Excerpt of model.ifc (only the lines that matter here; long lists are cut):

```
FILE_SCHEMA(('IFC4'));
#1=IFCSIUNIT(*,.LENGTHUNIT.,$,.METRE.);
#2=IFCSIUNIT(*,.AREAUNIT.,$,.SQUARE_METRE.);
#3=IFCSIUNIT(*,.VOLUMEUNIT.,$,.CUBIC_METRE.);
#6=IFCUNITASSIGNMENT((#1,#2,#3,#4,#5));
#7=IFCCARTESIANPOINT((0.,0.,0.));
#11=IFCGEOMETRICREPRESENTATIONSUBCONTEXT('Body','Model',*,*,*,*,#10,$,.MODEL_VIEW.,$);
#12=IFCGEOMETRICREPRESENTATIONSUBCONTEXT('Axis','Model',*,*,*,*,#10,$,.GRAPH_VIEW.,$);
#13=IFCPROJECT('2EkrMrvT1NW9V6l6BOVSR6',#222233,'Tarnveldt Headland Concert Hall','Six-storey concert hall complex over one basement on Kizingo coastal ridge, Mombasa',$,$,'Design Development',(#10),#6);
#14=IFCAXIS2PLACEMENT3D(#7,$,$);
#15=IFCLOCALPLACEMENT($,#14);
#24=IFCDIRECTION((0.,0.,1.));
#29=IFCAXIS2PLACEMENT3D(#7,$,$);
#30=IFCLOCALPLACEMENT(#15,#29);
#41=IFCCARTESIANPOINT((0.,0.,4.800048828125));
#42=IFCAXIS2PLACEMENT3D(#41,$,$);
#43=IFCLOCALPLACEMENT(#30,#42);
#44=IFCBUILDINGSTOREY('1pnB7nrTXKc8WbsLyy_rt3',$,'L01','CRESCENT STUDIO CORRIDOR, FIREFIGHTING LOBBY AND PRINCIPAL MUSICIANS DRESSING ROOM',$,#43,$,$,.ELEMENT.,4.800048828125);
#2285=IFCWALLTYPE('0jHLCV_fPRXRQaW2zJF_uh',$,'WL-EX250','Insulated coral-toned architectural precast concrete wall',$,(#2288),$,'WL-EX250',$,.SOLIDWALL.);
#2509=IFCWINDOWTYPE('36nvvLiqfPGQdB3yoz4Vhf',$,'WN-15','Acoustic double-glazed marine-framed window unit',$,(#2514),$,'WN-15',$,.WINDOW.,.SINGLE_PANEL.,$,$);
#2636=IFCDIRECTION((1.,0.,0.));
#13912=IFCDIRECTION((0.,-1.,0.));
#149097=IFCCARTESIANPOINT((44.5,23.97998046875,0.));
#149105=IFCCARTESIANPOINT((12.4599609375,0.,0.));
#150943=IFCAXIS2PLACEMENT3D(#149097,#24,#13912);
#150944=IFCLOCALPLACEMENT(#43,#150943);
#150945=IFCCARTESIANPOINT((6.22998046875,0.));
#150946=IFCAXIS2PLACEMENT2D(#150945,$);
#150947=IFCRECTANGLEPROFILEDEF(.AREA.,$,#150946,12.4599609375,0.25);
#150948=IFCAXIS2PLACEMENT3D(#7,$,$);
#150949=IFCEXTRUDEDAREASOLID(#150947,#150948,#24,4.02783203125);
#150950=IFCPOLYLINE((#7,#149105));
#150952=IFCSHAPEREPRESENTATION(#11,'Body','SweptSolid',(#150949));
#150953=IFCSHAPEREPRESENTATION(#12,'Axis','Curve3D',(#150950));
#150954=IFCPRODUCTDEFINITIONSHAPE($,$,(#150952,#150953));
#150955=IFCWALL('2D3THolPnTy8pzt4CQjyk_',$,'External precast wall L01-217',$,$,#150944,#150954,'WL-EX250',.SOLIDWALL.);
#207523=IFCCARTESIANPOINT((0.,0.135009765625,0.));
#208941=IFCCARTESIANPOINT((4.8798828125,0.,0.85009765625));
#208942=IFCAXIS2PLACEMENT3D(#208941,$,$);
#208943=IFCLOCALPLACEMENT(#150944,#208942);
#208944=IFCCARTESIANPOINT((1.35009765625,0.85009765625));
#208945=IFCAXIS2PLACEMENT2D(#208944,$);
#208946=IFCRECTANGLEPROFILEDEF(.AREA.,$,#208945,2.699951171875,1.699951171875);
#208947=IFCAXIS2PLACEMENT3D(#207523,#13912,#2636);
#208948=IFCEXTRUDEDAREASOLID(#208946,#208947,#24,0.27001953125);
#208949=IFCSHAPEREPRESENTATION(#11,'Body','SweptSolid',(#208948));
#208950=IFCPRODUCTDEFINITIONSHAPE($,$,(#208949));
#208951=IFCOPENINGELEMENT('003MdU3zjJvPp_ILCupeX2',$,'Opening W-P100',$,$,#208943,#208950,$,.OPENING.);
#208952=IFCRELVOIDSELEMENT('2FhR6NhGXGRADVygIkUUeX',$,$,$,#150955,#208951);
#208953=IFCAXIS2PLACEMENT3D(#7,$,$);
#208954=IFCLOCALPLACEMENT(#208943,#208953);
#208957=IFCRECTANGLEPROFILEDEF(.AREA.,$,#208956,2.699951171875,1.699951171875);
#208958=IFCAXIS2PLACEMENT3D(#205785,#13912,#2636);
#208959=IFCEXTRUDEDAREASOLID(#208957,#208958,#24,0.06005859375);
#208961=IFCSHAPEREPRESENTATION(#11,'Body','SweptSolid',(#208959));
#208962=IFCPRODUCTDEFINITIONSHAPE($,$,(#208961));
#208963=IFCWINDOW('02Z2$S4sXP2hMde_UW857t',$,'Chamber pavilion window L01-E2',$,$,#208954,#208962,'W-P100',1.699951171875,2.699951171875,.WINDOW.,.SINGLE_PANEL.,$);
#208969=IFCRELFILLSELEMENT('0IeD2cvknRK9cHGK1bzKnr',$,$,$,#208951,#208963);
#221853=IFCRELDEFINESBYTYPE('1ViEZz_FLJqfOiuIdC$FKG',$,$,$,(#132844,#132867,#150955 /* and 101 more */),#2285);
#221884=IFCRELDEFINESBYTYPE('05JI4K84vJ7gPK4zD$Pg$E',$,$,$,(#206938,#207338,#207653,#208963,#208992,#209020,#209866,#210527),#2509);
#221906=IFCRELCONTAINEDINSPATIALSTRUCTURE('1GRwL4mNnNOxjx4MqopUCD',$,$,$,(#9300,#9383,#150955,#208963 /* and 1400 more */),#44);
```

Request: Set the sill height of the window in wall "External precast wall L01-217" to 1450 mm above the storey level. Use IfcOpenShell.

```python
import numpy as np
import ifcopenshell
import ifcopenshell.api.geometry
import ifcopenshell.geom
import ifcopenshell.util.element
import ifcopenshell.util.placement
import ifcopenshell.util.shape
import ifcopenshell.util.unit

model = ifcopenshell.open("model.ifc")
unit_scale = ifcopenshell.util.unit.calculate_unit_scale(model)

window = model.by_guid("02Z2$S4sXP2hMde_UW857t")
opening = window.FillsVoids[0].RelatingOpeningElement
storey = ifcopenshell.util.element.get_container(window, ifc_class="IfcBuildingStorey")
level = ifcopenshell.util.placement.get_local_placement(storey.ObjectPlacement)[2, 3]

# The opening's origin need not be at the sill, so measure its lowest point.
shape = ifcopenshell.geom.create_shape(ifcopenshell.geom.settings(), opening)
bottom = ifcopenshell.util.shape.get_shape_bottom_elevation(shape, shape.geometry) / unit_scale
dz = level + 1.45 / unit_scale - bottom

shift = np.array([0.0, 0.0, dz])
# The window is placed relative to its opening, so it follows when the opening moves.
matrix = ifcopenshell.util.placement.get_local_placement(opening.ObjectPlacement)
matrix[:3, 3] += shift
ifcopenshell.api.geometry.edit_object_placement(
    model, product=opening, matrix=matrix, is_si=False, should_transform_children=True
)

print(f"moved by {dz * unit_scale:+.3f} m")

model.write("model_v2.ifc")
```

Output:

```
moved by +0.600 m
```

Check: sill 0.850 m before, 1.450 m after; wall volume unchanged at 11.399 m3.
